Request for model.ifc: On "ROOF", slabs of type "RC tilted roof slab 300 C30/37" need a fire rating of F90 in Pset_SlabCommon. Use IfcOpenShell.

First a look at what the model holds.

```python
import ifcopenshell
import ifcopenshell.util.element

model = ifcopenshell.open("model.ifc")
print(model.schema)
storey = next(s for s in model.by_type("IfcBuildingStorey") if s.Name == "ROOF")
slabs = [e for e in ifcopenshell.util.element.get_decomposition(storey) if e.is_a("IfcSlab")]
seen = {}
for e in slabs:
    element_type = ifcopenshell.util.element.get_type(e)
    key = (element_type.Name if element_type != e and element_type else None, ifcopenshell.util.element.get_pset(e, "Pset_SlabCommon", "FireRating"))
    seen[key] = seen.get(key, 0) + 1
for (name, value), count in sorted(seen.items(), key=str):
    print(count, "x", name, "|", value)
```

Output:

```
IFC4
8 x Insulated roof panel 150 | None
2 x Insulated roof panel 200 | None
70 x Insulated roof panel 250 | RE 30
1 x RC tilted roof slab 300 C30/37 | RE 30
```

```python
import ifcopenshell
import ifcopenshell.api.pset
import ifcopenshell.util.element

model = ifcopenshell.open("model.ifc")

storey = next(s for s in model.by_type("IfcBuildingStorey") if s.Name == "ROOF")
slabs = [e for e in ifcopenshell.util.element.get_decomposition(storey) if e.is_a("IfcSlab")]

count = 0
for e in slabs:
    element_type = ifcopenshell.util.element.get_type(e)
    if element_type in (None, e) or element_type.Name != "RC tilted roof slab 300 C30/37":
        continue
    # add_pset returns the element's existing set when there is one.
    pset = ifcopenshell.api.pset.add_pset(model, product=e, name="Pset_SlabCommon")
    ifcopenshell.api.pset.edit_pset(model, pset=pset, properties={"FireRating": "F90"})
    count += 1

print(count, "slabs updated")

model.write("model-out.ifc")
```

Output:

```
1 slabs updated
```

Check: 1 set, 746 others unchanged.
